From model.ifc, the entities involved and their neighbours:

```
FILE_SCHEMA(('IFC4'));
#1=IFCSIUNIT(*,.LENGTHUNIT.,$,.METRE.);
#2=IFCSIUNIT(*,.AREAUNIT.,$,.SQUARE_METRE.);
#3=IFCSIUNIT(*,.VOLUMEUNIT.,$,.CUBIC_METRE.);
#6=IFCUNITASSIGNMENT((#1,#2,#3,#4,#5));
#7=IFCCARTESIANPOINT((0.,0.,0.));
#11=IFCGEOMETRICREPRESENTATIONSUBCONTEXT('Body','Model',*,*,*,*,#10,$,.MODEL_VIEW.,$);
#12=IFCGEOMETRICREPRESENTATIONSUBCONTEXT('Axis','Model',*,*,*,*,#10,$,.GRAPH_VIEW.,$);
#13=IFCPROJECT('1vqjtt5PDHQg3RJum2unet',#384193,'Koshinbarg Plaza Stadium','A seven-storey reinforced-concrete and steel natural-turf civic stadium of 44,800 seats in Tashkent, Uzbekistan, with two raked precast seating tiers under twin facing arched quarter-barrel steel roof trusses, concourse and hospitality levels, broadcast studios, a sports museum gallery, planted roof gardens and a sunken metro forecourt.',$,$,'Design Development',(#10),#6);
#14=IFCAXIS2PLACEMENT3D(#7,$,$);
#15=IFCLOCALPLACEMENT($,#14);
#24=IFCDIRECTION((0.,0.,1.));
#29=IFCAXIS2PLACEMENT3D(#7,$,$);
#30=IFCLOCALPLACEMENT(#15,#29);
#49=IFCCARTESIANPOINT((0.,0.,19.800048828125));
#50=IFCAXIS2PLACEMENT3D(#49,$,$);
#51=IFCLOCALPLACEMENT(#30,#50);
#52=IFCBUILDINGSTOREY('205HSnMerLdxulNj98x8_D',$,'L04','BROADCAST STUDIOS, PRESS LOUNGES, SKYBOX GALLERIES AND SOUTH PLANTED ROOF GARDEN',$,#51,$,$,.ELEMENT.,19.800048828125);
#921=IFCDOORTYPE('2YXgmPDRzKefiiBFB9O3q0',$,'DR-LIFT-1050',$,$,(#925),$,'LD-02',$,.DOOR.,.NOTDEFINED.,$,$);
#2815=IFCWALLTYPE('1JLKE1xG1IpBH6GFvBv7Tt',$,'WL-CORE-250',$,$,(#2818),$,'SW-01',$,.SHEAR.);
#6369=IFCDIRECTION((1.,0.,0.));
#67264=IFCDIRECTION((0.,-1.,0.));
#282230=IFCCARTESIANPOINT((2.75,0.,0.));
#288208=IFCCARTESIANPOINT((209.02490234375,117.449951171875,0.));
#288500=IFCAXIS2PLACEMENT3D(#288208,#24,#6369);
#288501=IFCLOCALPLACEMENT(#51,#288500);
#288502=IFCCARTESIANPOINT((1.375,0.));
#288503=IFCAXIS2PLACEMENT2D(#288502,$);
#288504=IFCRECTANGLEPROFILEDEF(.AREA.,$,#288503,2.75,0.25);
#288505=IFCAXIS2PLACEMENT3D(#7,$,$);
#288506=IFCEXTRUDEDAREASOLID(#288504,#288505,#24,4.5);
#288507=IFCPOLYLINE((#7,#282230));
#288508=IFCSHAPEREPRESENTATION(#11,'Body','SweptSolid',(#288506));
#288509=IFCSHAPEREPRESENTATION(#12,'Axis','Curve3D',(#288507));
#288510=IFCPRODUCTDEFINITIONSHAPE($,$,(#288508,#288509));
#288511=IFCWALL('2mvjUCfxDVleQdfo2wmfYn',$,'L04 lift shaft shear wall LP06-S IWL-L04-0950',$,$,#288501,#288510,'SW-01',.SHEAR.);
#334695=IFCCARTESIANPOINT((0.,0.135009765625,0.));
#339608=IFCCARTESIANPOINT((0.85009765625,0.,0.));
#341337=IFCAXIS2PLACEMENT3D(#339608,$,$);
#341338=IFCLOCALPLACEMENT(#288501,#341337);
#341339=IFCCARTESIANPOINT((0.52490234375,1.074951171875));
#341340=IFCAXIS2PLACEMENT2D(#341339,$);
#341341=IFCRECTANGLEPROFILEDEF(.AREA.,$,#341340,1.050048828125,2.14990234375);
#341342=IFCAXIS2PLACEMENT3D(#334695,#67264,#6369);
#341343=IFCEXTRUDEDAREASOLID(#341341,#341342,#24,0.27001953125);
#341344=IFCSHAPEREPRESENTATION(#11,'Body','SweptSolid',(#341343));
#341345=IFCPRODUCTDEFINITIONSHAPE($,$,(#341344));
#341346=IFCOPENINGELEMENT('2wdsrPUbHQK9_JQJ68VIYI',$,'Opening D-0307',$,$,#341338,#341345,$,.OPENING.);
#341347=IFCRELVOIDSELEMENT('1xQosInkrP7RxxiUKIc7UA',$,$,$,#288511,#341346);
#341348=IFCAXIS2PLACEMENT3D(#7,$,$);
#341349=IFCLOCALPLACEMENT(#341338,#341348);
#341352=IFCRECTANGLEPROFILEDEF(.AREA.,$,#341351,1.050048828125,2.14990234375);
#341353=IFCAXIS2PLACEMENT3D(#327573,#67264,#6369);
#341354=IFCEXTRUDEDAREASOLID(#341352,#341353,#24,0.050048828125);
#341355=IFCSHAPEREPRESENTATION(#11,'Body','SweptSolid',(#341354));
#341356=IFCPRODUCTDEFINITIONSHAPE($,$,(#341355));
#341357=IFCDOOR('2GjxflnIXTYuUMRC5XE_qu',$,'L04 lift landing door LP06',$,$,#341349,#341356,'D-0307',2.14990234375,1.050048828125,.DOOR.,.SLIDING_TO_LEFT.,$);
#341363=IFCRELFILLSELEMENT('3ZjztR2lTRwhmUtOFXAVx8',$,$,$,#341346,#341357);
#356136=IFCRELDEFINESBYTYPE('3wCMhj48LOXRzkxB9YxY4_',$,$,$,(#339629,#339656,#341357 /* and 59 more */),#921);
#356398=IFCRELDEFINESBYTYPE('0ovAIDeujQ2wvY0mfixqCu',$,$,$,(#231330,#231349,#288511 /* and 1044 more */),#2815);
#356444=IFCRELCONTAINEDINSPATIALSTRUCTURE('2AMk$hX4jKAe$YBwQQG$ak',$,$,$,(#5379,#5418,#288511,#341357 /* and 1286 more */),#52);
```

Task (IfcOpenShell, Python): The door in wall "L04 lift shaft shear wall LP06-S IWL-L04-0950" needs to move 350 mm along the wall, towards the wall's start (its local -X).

```python
import ifcopenshell
import ifcopenshell.api.geometry
import ifcopenshell.util.placement
import ifcopenshell.util.unit

model = ifcopenshell.open("model.ifc")
unit_scale = ifcopenshell.util.unit.calculate_unit_scale(model)

door = model.by_guid("2GjxflnIXTYuUMRC5XE_qu")
opening = door.FillsVoids[0].RelatingOpeningElement
wall = opening.VoidsElements[0].RelatingBuildingElement

wall_matrix = ifcopenshell.util.placement.get_local_placement(wall.ObjectPlacement)
shift = wall_matrix[:3, 0] * -0.35 / unit_scale
before = ifcopenshell.util.placement.get_local_placement(door.ObjectPlacement)[:3, 3].copy()

# The door is placed relative to its opening, so it follows when the opening moves.
matrix = ifcopenshell.util.placement.get_local_placement(opening.ObjectPlacement)
matrix[:3, 3] += shift
ifcopenshell.api.geometry.edit_object_placement(
    model, product=opening, matrix=matrix, is_si=False, should_transform_children=True
)

after = ifcopenshell.util.placement.get_local_placement(door.ObjectPlacement)[:3, 3]
print("door moved by", (after - before).round(3) + 0.0)

model.write("model_rev.ifc")
```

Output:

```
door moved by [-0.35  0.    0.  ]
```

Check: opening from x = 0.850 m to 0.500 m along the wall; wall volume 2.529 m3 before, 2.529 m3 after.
